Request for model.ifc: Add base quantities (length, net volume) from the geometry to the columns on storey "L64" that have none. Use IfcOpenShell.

First a look at what the model holds.

```python
import ifcopenshell
import ifcopenshell.util.element
import ifcopenshell.util.unit

model = ifcopenshell.open("model.ifc")
print(model.schema)
for unit_type in ("LENGTHUNIT", "AREAUNIT", "VOLUMEUNIT"):
    print(unit_type, ifcopenshell.util.unit.calculate_unit_scale(model, unit_type))
storey = next(s for s in model.by_type("IfcBuildingStorey") if s.Name == "L64")
columns = [e for e in ifcopenshell.util.element.get_decomposition(storey) if e.is_a("IfcColumn")]
for e in sorted(columns, key=lambda e: e.id()):
    print(e.id(), e.is_a(), e.Name, list(ifcopenshell.util.element.get_psets(e, qtos_only=True)), sep=" | ")
```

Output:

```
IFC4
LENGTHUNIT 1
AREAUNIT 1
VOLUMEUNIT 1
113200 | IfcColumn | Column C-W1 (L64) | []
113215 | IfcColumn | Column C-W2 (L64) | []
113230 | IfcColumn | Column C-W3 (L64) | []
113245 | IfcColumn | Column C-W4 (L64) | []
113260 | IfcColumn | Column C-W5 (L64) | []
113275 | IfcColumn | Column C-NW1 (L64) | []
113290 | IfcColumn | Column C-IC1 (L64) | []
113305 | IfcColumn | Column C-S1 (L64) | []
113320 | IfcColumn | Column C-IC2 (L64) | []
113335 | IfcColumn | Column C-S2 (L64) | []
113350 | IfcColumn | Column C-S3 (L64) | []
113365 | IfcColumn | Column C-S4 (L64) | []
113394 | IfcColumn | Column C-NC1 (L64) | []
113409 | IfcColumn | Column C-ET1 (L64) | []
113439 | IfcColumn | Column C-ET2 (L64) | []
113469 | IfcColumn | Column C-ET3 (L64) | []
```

```python
import ifcopenshell
import ifcopenshell.api.pset
import ifcopenshell.geom
import ifcopenshell.util.element
import ifcopenshell.util.shape
import ifcopenshell.util.unit

model = ifcopenshell.open("model.ifc")
unit_scale = ifcopenshell.util.unit.calculate_unit_scale(model)
volume_scale = ifcopenshell.util.unit.calculate_unit_scale(model, "VOLUMEUNIT")
settings = ifcopenshell.geom.settings()

storey = next(s for s in model.by_type("IfcBuildingStorey") if s.Name == "L64")
columns = [e for e in ifcopenshell.util.element.get_decomposition(storey) if e.is_a("IfcColumn")]

for e in sorted(columns, key=lambda e: e.id()):
    if ifcopenshell.util.element.get_psets(e, qtos_only=True, should_inherit=False):
        continue
    # Geometry comes back in metres, in the element's own axes.
    shape = ifcopenshell.geom.create_shape(settings, e)
    values = {
        "Length": ifcopenshell.util.shape.get_z(shape.geometry) / unit_scale,
        "NetVolume": ifcopenshell.util.shape.get_volume(shape.geometry) / volume_scale,
    }
    qto = ifcopenshell.api.pset.add_qto(model, product=e, name="Qto_ColumnBaseQuantities")
    ifcopenshell.api.pset.edit_qto(model, qto=qto, properties=values)
    print(e.id(), {k: round(v, 3) for k, v in values.items()})

model.write("model_edited.ifc")
```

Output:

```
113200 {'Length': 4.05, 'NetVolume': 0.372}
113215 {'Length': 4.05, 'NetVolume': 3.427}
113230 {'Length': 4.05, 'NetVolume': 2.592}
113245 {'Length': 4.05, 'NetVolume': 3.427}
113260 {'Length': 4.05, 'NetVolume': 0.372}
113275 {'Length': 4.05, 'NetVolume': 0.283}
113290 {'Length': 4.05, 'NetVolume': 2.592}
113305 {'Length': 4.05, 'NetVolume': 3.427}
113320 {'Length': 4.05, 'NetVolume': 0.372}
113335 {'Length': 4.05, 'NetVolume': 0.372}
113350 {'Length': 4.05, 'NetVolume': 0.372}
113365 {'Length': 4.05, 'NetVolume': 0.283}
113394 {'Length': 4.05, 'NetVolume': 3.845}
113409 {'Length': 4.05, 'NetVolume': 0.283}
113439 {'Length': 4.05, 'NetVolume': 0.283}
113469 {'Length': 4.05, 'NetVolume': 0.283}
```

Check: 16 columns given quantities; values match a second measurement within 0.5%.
